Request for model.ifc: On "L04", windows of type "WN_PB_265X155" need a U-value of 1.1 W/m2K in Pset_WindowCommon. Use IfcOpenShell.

First a look at what the model holds.

```python
import ifcopenshell
import ifcopenshell.util.element

model = ifcopenshell.open("model.ifc")
print(model.schema)
storey = next(s for s in model.by_type("IfcBuildingStorey") if s.Name == "L04")
windows = [e for e in ifcopenshell.util.element.get_decomposition(storey) if e.is_a("IfcWindow")]
seen = {}
for e in windows:
    element_type = ifcopenshell.util.element.get_type(e)
    key = (element_type.Name if element_type != e and element_type else None, ifcopenshell.util.element.get_pset(e, "Pset_WindowCommon", "ThermalTransmittance"))
    seen[key] = seen.get(key, 0) + 1
for (name, value), count in sorted(seen.items(), key=str):
    print(count, "x", name, "|", value)
```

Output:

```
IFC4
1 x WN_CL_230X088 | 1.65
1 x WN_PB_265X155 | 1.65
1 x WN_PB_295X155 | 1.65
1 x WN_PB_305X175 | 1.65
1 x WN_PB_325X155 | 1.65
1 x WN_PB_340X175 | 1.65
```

```python
import ifcopenshell
import ifcopenshell.api.pset
import ifcopenshell.util.element

model = ifcopenshell.open("model.ifc")

storey = next(s for s in model.by_type("IfcBuildingStorey") if s.Name == "L04")
windows = [e for e in ifcopenshell.util.element.get_decomposition(storey) if e.is_a("IfcWindow")]

count = 0
for e in windows:
    element_type = ifcopenshell.util.element.get_type(e)
    if element_type in (None, e) or element_type.Name != "WN_PB_265X155":
        continue
    # add_pset returns the element's existing set when there is one.
    pset = ifcopenshell.api.pset.add_pset(model, product=e, name="Pset_WindowCommon")
    ifcopenshell.api.pset.edit_pset(model, pset=pset, properties={"ThermalTransmittance": 1.1})
    count += 1

print(count, "windows updated")

model.write("model-out.ifc")
```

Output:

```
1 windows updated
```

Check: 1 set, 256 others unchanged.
